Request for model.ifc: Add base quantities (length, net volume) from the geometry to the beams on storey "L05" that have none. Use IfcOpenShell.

First a look at what the model holds.

```python
import ifcopenshell
import ifcopenshell.util.element
import ifcopenshell.util.unit

model = ifcopenshell.open("model.ifc")
print(model.schema)
for unit_type in ("LENGTHUNIT", "AREAUNIT", "VOLUMEUNIT"):
    print(unit_type, ifcopenshell.util.unit.calculate_unit_scale(model, unit_type))
storey = next(s for s in model.by_type("IfcBuildingStorey") if s.Name == "L05")
beams = [e for e in ifcopenshell.util.element.get_decomposition(storey) if e.is_a("IfcBeam")]
for e in sorted(beams, key=lambda e: e.id()):
    print(e.id(), e.is_a(), e.Name, list(ifcopenshell.util.element.get_psets(e, qtos_only=True)), sep=" | ")
```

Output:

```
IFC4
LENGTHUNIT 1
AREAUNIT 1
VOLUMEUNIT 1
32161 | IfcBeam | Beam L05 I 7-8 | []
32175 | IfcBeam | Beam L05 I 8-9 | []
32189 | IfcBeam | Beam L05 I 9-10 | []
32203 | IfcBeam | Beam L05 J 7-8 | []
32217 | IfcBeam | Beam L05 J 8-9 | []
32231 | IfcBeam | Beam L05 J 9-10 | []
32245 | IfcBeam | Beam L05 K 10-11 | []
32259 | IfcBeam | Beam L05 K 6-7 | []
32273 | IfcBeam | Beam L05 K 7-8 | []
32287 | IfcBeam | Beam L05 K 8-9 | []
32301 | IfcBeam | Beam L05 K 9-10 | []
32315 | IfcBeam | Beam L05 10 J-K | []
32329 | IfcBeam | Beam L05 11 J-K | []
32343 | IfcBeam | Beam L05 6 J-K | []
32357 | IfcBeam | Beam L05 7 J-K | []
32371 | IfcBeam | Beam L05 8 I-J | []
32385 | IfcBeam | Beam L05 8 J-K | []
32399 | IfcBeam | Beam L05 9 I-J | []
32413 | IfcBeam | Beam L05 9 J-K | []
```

```python
import ifcopenshell
import ifcopenshell.api.pset
import ifcopenshell.geom
import ifcopenshell.util.element
import ifcopenshell.util.shape
import ifcopenshell.util.unit

model = ifcopenshell.open("model.ifc")
unit_scale = ifcopenshell.util.unit.calculate_unit_scale(model)
volume_scale = ifcopenshell.util.unit.calculate_unit_scale(model, "VOLUMEUNIT")
settings = ifcopenshell.geom.settings()

storey = next(s for s in model.by_type("IfcBuildingStorey") if s.Name == "L05")
beams = [e for e in ifcopenshell.util.element.get_decomposition(storey) if e.is_a("IfcBeam")]

for e in sorted(beams, key=lambda e: e.id()):
    if ifcopenshell.util.element.get_psets(e, qtos_only=True, should_inherit=False):
        continue
    # Geometry comes back in metres, in the element's own axes.
    shape = ifcopenshell.geom.create_shape(settings, e)
    values = {
        "Length": ifcopenshell.util.shape.get_max_xyz(shape.geometry) / unit_scale,
        "NetVolume": ifcopenshell.util.shape.get_volume(shape.geometry) / volume_scale,
    }
    qto = ifcopenshell.api.pset.add_qto(model, product=e, name="Qto_BeamBaseQuantities")
    ifcopenshell.api.pset.edit_qto(model, qto=qto, properties=values)
    print(e.id(), {k: round(v, 3) for k, v in values.items()})

model.write("model_edited.ifc")
```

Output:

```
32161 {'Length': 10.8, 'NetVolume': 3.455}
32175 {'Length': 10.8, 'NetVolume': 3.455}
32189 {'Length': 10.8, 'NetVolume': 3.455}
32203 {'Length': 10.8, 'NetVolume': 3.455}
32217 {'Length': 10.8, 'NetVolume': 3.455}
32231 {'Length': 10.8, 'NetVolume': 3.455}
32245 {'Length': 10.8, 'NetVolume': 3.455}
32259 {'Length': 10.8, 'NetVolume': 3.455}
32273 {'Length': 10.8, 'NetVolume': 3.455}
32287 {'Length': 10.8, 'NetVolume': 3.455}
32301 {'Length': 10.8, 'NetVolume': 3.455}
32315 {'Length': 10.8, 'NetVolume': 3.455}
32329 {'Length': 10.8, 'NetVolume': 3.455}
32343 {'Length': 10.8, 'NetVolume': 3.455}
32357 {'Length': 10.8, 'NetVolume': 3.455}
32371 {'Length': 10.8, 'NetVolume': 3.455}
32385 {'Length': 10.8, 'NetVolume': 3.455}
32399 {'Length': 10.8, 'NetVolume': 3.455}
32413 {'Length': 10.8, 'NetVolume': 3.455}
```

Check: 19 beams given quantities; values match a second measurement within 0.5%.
